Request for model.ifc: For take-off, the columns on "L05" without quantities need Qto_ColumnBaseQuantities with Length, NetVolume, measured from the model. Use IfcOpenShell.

First a look at what the model holds.

```python
import ifcopenshell
import ifcopenshell.util.element
import ifcopenshell.util.unit

model = ifcopenshell.open("model.ifc")
print(model.schema)
for unit_type in ("LENGTHUNIT", "AREAUNIT", "VOLUMEUNIT"):
    print(unit_type, ifcopenshell.util.unit.calculate_unit_scale(model, unit_type))
storey = next(s for s in model.by_type("IfcBuildingStorey") if s.Name == "L05")
columns = [e for e in ifcopenshell.util.element.get_decomposition(storey) if e.is_a("IfcColumn")]
for e in sorted(columns, key=lambda e: e.id()):
    print(e.id(), e.is_a(), e.Name, list(ifcopenshell.util.element.get_psets(e, qtos_only=True)), sep=" | ")
```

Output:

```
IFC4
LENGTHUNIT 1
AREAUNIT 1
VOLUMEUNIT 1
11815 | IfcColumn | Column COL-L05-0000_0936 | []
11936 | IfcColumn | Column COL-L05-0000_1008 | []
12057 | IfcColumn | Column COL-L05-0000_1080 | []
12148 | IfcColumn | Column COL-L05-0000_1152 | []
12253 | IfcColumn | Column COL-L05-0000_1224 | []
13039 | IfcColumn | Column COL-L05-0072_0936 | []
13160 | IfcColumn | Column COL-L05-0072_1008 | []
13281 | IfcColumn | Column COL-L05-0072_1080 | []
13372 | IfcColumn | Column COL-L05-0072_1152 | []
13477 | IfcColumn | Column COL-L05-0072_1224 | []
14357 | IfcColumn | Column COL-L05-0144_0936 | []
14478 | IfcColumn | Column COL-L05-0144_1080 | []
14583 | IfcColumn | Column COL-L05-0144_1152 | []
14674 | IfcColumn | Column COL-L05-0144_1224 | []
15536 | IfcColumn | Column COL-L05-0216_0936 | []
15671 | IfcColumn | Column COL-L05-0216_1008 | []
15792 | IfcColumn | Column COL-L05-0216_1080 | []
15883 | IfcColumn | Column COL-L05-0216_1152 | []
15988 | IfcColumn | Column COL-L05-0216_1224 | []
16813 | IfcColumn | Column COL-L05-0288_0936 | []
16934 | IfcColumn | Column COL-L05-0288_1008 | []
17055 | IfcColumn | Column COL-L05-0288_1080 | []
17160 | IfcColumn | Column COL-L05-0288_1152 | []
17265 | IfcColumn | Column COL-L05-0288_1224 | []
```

```python
import ifcopenshell
import ifcopenshell.api.pset
import ifcopenshell.geom
import ifcopenshell.util.element
import ifcopenshell.util.shape
import ifcopenshell.util.unit

model = ifcopenshell.open("model.ifc")
unit_scale = ifcopenshell.util.unit.calculate_unit_scale(model)
volume_scale = ifcopenshell.util.unit.calculate_unit_scale(model, "VOLUMEUNIT")
settings = ifcopenshell.geom.settings()

storey = next(s for s in model.by_type("IfcBuildingStorey") if s.Name == "L05")
columns = [e for e in ifcopenshell.util.element.get_decomposition(storey) if e.is_a("IfcColumn")]

for e in sorted(columns, key=lambda e: e.id()):
    if ifcopenshell.util.element.get_psets(e, qtos_only=True, should_inherit=False):
        continue
    # Geometry comes back in metres, in the element's own axes.
    shape = ifcopenshell.geom.create_shape(settings, e)
    values = {
        "Length": ifcopenshell.util.shape.get_z(shape.geometry) / unit_scale,
        "NetVolume": ifcopenshell.util.shape.get_volume(shape.geometry) / volume_scale,
    }
    qto = ifcopenshell.api.pset.add_qto(model, product=e, name="Qto_ColumnBaseQuantities")
    ifcopenshell.api.pset.edit_qto(model, qto=qto, properties=values)
    print(e.id(), {k: round(v, 3) for k, v in values.items()})

model.write("model_rev.ifc")
```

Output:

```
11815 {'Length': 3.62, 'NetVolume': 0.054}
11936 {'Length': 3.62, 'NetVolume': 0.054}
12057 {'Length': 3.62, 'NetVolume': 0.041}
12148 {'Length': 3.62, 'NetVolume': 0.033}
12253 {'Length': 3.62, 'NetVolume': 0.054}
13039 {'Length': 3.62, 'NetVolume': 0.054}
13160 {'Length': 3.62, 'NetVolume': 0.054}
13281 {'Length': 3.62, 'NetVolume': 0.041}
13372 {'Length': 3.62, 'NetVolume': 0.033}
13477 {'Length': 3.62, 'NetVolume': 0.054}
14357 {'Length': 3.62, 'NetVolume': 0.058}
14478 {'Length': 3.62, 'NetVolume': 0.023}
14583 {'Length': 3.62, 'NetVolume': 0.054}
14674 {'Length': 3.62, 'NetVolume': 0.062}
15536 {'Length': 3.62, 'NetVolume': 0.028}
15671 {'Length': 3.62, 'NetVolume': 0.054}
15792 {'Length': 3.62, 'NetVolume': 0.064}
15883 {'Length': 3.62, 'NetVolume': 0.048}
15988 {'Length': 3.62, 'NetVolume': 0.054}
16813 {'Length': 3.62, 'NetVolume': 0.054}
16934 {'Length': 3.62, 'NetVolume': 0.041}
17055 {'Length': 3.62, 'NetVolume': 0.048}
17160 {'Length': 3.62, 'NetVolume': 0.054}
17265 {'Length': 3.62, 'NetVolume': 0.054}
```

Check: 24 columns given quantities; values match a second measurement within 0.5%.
